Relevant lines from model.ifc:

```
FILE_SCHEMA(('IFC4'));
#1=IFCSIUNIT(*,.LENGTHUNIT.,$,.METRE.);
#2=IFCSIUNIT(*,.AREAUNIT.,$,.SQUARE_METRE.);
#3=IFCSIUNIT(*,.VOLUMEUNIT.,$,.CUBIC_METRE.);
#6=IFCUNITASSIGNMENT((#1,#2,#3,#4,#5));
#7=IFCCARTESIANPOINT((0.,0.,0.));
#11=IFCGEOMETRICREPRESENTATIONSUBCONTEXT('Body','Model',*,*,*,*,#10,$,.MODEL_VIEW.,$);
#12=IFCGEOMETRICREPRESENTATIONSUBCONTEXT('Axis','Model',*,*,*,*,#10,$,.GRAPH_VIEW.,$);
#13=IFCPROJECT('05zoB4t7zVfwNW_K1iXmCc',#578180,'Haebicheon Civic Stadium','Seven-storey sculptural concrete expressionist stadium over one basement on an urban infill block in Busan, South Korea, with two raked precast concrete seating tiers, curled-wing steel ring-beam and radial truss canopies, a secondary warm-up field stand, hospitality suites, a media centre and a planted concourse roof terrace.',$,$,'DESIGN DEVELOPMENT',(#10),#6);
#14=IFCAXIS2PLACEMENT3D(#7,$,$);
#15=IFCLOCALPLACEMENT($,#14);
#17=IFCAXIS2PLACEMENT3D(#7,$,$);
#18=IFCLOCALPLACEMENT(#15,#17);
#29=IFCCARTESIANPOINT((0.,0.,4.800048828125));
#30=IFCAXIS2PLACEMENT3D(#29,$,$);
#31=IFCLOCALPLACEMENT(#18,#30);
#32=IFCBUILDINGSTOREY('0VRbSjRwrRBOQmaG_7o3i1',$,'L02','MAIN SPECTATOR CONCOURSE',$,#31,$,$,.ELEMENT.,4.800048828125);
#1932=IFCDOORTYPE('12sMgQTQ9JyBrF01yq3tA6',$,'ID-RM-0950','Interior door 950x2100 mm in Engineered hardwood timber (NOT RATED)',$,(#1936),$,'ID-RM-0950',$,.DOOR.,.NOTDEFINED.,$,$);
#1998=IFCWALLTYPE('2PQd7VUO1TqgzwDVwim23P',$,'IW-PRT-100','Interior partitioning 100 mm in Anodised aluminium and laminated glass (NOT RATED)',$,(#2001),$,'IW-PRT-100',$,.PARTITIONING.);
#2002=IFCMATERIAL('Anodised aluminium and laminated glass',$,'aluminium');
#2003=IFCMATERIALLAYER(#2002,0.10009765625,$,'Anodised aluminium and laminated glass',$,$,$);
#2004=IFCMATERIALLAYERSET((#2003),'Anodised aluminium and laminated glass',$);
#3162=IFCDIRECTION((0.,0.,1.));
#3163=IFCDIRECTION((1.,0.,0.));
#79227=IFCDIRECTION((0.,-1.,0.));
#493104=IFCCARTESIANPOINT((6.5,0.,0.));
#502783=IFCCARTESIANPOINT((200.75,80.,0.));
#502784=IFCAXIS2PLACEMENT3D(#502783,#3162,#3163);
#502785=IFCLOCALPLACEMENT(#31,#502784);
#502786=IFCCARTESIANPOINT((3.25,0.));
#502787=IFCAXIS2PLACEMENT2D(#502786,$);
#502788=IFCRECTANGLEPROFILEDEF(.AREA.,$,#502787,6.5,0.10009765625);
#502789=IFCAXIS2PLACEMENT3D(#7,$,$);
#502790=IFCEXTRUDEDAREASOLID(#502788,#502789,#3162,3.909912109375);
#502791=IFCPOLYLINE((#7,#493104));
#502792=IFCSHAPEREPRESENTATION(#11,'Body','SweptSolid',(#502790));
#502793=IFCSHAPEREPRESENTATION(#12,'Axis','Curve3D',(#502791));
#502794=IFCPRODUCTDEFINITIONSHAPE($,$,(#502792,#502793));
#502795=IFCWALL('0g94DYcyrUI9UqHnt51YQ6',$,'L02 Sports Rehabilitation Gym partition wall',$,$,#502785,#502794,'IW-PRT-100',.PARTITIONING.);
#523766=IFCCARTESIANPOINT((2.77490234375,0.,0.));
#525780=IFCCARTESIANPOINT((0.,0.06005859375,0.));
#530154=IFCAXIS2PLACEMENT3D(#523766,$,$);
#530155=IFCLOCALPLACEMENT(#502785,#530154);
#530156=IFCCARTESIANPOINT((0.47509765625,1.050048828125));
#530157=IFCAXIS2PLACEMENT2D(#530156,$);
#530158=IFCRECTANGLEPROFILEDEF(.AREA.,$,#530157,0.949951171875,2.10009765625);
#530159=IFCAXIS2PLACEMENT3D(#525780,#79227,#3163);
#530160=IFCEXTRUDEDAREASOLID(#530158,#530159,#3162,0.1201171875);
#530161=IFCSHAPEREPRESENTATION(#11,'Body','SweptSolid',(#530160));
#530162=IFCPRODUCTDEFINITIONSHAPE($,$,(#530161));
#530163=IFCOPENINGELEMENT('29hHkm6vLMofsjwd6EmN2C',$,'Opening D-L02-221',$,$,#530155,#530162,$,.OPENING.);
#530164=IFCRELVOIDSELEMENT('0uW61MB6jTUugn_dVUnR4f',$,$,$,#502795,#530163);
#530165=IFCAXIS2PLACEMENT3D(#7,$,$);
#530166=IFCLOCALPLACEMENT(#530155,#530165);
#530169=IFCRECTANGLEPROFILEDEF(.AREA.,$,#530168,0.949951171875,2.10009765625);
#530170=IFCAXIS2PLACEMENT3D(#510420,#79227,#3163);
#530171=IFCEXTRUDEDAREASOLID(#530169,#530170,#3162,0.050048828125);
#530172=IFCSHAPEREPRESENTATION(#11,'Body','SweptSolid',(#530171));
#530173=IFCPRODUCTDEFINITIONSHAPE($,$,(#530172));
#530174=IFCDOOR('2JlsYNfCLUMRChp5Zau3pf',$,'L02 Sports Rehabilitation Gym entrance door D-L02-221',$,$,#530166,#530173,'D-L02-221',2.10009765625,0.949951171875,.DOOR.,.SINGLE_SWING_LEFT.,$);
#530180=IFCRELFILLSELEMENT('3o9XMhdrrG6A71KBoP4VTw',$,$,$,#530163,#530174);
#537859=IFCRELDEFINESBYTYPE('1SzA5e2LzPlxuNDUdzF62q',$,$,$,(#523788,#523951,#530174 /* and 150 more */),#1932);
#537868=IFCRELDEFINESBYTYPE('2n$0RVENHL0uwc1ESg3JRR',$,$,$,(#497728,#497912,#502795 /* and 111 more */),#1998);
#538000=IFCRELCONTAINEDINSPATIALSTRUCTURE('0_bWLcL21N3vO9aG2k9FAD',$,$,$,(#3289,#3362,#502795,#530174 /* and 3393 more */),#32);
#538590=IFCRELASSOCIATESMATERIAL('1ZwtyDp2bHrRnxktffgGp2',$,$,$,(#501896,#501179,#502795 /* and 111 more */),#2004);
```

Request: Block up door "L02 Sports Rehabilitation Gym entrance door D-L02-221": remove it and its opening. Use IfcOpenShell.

```python
import ifcopenshell
import ifcopenshell.api.feature
import ifcopenshell.api.root
import ifcopenshell.geom
import ifcopenshell.util.shape

model = ifcopenshell.open("model.ifc")
settings = ifcopenshell.geom.settings()


def volume(element):
    """Net volume in cubic metres, openings subtracted."""
    shape = ifcopenshell.geom.create_shape(settings, element)
    return ifcopenshell.util.shape.get_volume(shape.geometry)


door = model.by_guid("2JlsYNfCLUMRChp5Zau3pf")
opening = door.FillsVoids[0].RelatingOpeningElement
wall = opening.VoidsElements[0].RelatingBuildingElement
before = volume(wall)

ifcopenshell.api.root.remove_product(model, product=door)
ifcopenshell.api.feature.remove_feature(model, feature=opening)

after = volume(wall)

print(f"wall volume {before:.3f} -> {after:.3f} m3")

model.write("model_rev.ifc")
```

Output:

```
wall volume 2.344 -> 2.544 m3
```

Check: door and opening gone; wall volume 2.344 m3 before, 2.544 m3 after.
